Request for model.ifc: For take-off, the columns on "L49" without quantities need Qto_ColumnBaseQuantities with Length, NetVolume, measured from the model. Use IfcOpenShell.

First a look at what the model holds.

```python
import ifcopenshell
import ifcopenshell.util.element
import ifcopenshell.util.unit

model = ifcopenshell.open("model.ifc")
print(model.schema)
for unit_type in ("LENGTHUNIT", "AREAUNIT", "VOLUMEUNIT"):
    print(unit_type, ifcopenshell.util.unit.calculate_unit_scale(model, unit_type))
storey = next(s for s in model.by_type("IfcBuildingStorey") if s.Name == "L49")
columns = [e for e in ifcopenshell.util.element.get_decomposition(storey) if e.is_a("IfcColumn")]
for e in sorted(columns, key=lambda e: e.id()):
    print(e.id(), e.is_a(), e.Name, list(ifcopenshell.util.element.get_psets(e, qtos_only=True)), sep=" | ")
```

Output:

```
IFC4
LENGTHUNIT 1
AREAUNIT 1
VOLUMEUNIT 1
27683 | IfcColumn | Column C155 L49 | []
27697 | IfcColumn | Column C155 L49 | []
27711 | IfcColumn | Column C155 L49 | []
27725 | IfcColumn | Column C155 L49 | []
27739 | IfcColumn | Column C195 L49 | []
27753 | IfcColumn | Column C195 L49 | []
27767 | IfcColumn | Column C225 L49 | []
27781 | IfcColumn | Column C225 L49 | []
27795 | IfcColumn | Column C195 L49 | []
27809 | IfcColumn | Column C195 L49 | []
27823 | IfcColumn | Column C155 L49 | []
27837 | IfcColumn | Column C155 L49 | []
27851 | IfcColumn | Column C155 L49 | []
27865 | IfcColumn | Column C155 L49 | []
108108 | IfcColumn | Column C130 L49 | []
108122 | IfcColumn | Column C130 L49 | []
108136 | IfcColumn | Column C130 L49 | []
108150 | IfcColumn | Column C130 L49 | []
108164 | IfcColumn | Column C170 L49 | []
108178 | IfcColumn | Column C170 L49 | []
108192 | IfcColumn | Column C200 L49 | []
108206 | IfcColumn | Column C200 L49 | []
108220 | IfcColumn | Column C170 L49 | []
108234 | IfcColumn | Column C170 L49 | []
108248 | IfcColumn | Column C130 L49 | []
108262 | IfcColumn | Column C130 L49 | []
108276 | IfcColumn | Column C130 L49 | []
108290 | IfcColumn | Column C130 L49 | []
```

```python
import ifcopenshell
import ifcopenshell.api.pset
import ifcopenshell.geom
import ifcopenshell.util.element
import ifcopenshell.util.shape
import ifcopenshell.util.unit

model = ifcopenshell.open("model.ifc")
unit_scale = ifcopenshell.util.unit.calculate_unit_scale(model)
volume_scale = ifcopenshell.util.unit.calculate_unit_scale(model, "VOLUMEUNIT")
settings = ifcopenshell.geom.settings()

storey = next(s for s in model.by_type("IfcBuildingStorey") if s.Name == "L49")
columns = [e for e in ifcopenshell.util.element.get_decomposition(storey) if e.is_a("IfcColumn")]

for e in sorted(columns, key=lambda e: e.id()):
    if ifcopenshell.util.element.get_psets(e, qtos_only=True, should_inherit=False):
        continue
    # Geometry comes back in metres, in the element's own axes.
    shape = ifcopenshell.geom.create_shape(settings, e)
    values = {
        "Length": ifcopenshell.util.shape.get_z(shape.geometry) / unit_scale,
        "NetVolume": ifcopenshell.util.shape.get_volume(shape.geometry) / volume_scale,
    }
    qto = ifcopenshell.api.pset.add_qto(model, product=e, name="Qto_ColumnBaseQuantities")
    ifcopenshell.api.pset.edit_qto(model, qto=qto, properties=values)
    print(e.id(), {k: round(v, 3) for k, v in values.items()})

model.write("model_edited.ifc")
```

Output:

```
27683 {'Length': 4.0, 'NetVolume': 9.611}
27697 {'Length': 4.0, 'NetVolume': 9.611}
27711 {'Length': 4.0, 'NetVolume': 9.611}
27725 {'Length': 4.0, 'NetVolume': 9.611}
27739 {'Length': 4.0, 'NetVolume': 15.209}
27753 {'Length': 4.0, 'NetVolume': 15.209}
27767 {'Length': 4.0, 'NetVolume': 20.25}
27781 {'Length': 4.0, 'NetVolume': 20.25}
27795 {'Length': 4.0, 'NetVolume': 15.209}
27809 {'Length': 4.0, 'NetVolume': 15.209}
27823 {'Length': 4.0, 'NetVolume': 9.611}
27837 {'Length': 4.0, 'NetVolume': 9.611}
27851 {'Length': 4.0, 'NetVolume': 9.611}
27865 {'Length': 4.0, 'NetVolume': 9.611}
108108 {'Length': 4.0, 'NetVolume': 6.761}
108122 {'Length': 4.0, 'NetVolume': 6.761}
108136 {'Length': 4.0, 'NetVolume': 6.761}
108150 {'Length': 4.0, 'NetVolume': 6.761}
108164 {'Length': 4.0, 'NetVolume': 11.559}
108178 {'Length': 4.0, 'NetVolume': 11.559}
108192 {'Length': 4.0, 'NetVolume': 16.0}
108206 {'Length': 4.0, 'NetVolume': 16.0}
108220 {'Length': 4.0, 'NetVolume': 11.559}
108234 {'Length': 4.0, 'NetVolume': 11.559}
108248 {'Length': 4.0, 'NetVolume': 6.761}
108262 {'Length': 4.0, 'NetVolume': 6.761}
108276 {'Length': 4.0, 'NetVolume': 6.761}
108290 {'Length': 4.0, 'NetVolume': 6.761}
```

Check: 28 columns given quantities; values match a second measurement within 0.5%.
